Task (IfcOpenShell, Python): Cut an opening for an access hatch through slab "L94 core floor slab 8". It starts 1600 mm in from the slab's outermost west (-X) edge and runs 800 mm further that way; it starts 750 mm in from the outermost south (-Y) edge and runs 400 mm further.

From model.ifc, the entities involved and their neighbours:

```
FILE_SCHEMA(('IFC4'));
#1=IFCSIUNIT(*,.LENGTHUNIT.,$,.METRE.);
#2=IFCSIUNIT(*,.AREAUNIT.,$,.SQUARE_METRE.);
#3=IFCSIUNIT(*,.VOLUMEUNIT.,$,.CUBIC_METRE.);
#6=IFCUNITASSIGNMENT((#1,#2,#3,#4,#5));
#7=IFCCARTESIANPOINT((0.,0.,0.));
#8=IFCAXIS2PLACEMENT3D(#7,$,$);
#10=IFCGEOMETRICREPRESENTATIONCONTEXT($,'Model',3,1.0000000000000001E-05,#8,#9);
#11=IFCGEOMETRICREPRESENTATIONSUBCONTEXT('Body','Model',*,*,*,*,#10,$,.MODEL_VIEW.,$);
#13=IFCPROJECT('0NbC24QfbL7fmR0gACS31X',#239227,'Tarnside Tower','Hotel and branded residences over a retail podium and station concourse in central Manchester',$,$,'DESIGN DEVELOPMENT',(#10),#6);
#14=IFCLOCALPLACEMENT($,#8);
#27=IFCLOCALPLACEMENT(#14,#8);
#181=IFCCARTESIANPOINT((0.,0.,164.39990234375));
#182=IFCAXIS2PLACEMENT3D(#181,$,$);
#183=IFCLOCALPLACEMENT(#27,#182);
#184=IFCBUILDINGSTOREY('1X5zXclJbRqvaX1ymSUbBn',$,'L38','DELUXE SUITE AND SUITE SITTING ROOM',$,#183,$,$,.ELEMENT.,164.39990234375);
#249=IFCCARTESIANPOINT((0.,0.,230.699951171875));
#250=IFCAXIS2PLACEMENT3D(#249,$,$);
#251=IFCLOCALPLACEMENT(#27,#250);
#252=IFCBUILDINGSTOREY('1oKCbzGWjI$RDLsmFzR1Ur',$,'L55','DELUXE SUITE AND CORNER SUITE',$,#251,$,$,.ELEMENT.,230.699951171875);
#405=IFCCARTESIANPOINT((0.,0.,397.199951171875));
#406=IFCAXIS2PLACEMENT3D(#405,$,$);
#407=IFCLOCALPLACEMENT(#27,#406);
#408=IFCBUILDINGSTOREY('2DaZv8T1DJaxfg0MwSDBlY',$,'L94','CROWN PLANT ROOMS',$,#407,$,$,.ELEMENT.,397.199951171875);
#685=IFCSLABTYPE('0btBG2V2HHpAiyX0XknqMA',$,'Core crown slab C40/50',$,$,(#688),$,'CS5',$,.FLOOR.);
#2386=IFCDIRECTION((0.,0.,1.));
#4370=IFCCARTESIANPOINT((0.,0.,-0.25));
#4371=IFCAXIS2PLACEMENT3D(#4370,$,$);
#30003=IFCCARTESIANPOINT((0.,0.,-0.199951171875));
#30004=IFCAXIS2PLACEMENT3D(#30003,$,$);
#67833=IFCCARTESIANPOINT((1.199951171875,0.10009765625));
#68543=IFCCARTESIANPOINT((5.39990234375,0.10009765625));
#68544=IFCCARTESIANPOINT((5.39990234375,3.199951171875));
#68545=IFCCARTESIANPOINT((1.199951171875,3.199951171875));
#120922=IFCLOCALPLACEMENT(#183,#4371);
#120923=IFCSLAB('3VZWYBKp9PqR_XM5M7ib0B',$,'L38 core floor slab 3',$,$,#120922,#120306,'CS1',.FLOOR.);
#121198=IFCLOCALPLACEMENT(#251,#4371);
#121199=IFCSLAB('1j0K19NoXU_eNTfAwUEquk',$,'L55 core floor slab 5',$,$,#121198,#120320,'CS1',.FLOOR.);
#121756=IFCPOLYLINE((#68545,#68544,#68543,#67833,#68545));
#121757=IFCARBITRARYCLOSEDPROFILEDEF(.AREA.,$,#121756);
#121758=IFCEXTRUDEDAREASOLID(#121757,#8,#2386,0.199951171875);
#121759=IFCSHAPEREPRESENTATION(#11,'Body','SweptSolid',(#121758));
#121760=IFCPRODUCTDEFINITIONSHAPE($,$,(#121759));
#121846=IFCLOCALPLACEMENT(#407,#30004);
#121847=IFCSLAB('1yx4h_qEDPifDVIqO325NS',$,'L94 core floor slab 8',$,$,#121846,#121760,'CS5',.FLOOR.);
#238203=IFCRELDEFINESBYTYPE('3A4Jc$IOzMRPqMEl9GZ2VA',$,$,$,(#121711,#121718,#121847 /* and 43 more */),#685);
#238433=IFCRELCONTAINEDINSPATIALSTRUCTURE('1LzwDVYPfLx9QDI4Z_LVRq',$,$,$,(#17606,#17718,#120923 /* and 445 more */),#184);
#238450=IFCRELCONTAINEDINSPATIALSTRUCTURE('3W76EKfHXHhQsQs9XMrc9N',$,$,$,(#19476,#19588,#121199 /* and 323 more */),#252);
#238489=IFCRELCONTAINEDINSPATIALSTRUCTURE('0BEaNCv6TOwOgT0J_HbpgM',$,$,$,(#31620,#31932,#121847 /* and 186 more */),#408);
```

```python
import numpy as np
import ifcopenshell
import ifcopenshell.api.feature
import ifcopenshell.api.geometry
import ifcopenshell.api.root
import ifcopenshell.geom
import ifcopenshell.util.placement
import ifcopenshell.util.representation
import ifcopenshell.util.shape
import ifcopenshell.util.unit

model = ifcopenshell.open("model.ifc")
unit_scale = ifcopenshell.util.unit.calculate_unit_scale(model)
settings = ifcopenshell.geom.settings()


def volume(element):
    """Net volume in cubic metres, openings subtracted."""
    shape = ifcopenshell.geom.create_shape(settings, element)
    return ifcopenshell.util.shape.get_volume(shape.geometry)


slab = model.by_guid("1yx4h_qEDPifDVIqO325NS")
before = volume(slab)

# Extent in the slab's own axes, in metres. The edges named are its -X and -Y sides.
slab_shape = ifcopenshell.geom.create_shape(settings, slab)
vertices = ifcopenshell.util.shape.get_vertices(slab_shape.geometry)
x_min, y_min, bottom = vertices.min(axis=0)
top = vertices[:, 2].max()

opening = ifcopenshell.api.root.create_entity(model, ifc_class="IfcOpeningElement", name="Access hatch opening", predefined_type="OPENING")
context = ifcopenshell.util.representation.get_context(model, "Model", "Body", "MODEL_VIEW")
width, depth = 0.8, 0.4
outline = [(0.0, 0.0), (width, 0.0), (width, depth), (0.0, depth), (0.0, 0.0)]
# Overshoot both faces by 50 mm so the cut is clean.
shape = ifcopenshell.api.geometry.add_slab_representation(
    model, context=context, depth=top - bottom + 0.1, polyline=outline
)
ifcopenshell.api.geometry.assign_representation(model, product=opening, representation=shape)

matrix = ifcopenshell.util.placement.get_local_placement(slab.ObjectPlacement)
matrix[:, 3] = matrix @ np.append(np.array([x_min + 1.6, y_min + 0.75, bottom - 0.05]) / unit_scale, 1.0)
ifcopenshell.api.geometry.edit_object_placement(model, product=opening, matrix=matrix, is_si=False)
ifcopenshell.api.feature.add_feature(model, feature=opening, element=slab)

after = volume(slab)

print(f"slab volume {before:.3f} -> {after:.3f} m3")

model.write("model_updated.ifc")
```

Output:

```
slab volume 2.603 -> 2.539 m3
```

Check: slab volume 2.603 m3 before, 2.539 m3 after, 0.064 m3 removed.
